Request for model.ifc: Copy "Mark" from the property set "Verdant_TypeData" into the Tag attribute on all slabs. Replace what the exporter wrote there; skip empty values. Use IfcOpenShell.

First a look at what the model holds.

```python
import ifcopenshell
import ifcopenshell.util.element

model = ifcopenshell.open("model.ifc")
print(model.schema)
slabs = model.by_type("IfcSlab")
print(len(slabs), "slabs")
for e in slabs[:8]:
    source = ifcopenshell.util.element.get_pset(e, "Verdant_TypeData", "Mark")
    target = e.Tag
    print(e.id(), repr(source), repr(target), sep=" | ")
```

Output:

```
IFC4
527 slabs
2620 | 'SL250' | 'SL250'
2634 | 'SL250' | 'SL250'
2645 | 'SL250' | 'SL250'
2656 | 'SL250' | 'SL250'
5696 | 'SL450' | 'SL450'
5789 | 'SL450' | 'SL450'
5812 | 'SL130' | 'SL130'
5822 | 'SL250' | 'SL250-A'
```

```python
import ifcopenshell
import ifcopenshell.util.element

model = ifcopenshell.open("model.ifc")

count = 0
for e in model.by_type("IfcSlab"):
    value = ifcopenshell.util.element.get_pset(e, "Verdant_TypeData", "Mark")
    current = e.Tag
    if not value or not value.strip() or current == value:
        continue
    e.Tag = value
    count += 1

print(count, "slabs updated")

model.write("model_rev.ifc")
```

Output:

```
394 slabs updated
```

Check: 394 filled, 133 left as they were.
